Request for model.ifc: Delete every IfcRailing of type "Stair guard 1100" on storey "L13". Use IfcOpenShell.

First a look at what the model holds.

```python
import ifcopenshell
import ifcopenshell.util.element

model = ifcopenshell.open("model.ifc")
print(model.schema)
storey = next(s for s in model.by_type("IfcBuildingStorey") if s.Name == "L13")
railings = [e for e in ifcopenshell.util.element.get_decomposition(storey) if e.is_a("IfcRailing")]
seen = {}
for e in railings:
    element_type = ifcopenshell.util.element.get_type(e)
    name = element_type.Name if element_type not in (None, e) else None
    seen[name] = seen.get(name, 0) + 1
for name, count in sorted(seen.items(), key=str):
    print(count, "x", name)
```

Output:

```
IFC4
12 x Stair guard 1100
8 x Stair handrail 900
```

```python
import ifcopenshell
import ifcopenshell.api.root
import ifcopenshell.util.element

model = ifcopenshell.open("model.ifc")

storey = next(s for s in model.by_type("IfcBuildingStorey") if s.Name == "L13")
railings = [e for e in ifcopenshell.util.element.get_decomposition(storey) if e.is_a("IfcRailing")]
targets = [e for e in railings if (t := ifcopenshell.util.element.get_type(e)) not in (None, e) and t.Name == "Stair guard 1100"]

for e in targets:
    ifcopenshell.api.root.remove_product(model, product=e)
print(len(targets), "removed")

model.write("model_rev.ifc")
```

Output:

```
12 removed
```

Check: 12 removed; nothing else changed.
